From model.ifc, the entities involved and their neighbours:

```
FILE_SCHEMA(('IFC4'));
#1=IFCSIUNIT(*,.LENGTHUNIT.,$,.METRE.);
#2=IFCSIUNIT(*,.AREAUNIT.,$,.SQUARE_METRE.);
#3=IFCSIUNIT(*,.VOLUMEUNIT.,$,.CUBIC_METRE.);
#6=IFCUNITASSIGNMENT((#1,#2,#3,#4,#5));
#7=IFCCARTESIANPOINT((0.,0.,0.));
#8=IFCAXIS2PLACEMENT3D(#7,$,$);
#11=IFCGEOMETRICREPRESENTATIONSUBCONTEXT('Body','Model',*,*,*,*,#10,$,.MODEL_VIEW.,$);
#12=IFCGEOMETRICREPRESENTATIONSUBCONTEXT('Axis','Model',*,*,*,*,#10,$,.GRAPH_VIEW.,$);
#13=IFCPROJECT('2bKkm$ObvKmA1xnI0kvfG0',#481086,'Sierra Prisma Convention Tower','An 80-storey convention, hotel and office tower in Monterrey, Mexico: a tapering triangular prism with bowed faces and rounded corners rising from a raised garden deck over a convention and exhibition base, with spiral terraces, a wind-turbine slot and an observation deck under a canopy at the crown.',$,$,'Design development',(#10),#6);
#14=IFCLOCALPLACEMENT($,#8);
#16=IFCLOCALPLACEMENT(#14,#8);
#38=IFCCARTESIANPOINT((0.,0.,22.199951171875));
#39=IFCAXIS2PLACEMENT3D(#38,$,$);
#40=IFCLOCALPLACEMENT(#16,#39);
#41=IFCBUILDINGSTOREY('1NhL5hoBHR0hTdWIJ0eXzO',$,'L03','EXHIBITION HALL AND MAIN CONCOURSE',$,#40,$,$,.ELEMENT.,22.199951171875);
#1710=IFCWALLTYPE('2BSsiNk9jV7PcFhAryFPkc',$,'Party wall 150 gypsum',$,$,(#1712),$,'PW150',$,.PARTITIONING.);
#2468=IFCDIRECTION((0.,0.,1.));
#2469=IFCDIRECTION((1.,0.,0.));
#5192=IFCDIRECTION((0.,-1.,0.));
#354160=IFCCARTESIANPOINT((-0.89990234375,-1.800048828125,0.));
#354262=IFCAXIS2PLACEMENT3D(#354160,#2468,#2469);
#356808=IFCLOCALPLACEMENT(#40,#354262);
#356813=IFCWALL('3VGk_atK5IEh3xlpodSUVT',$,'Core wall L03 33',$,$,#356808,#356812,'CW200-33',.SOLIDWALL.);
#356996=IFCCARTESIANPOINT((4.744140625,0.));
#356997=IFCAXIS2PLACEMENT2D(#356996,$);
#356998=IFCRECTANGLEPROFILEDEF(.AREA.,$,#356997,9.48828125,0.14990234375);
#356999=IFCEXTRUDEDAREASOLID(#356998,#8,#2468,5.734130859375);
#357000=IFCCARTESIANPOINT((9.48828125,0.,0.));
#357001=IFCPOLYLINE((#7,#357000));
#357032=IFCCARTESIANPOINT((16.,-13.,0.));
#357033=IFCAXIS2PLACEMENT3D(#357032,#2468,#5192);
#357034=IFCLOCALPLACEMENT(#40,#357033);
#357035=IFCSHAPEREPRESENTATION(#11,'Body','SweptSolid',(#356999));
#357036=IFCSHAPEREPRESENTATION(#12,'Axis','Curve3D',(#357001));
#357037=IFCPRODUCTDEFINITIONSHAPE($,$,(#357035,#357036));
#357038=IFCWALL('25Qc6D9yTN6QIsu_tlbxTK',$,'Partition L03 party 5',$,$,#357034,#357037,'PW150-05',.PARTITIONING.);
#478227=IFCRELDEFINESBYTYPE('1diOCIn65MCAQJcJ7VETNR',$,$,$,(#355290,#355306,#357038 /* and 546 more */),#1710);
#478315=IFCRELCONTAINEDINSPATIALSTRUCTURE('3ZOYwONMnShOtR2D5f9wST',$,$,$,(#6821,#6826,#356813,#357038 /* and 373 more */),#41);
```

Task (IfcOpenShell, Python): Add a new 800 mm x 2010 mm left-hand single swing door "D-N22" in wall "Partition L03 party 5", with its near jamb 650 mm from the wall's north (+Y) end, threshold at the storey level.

```python
import numpy as np
import ifcopenshell
import ifcopenshell.api.feature
import ifcopenshell.api.geometry
import ifcopenshell.api.root
import ifcopenshell.api.spatial
import ifcopenshell.geom
import ifcopenshell.util.element
import ifcopenshell.util.placement
import ifcopenshell.util.representation
import ifcopenshell.util.shape
import ifcopenshell.util.unit

model = ifcopenshell.open("model.ifc")
unit_scale = ifcopenshell.util.unit.calculate_unit_scale(model)
settings = ifcopenshell.geom.settings()


def volume(element):
    """Net volume in cubic metres, openings subtracted."""
    shape = ifcopenshell.geom.create_shape(settings, element)
    return ifcopenshell.util.shape.get_volume(shape.geometry)


wall = model.by_guid("25Qc6D9yTN6QIsu_tlbxTK")
storey = ifcopenshell.util.element.get_container(wall, ifc_class="IfcBuildingStorey")
context = ifcopenshell.util.representation.get_context(model, "Model", "Body", "MODEL_VIEW")
before = volume(wall)

width, height, from_end, sill = 0.8, 2.01, 0.65, 0.0  # metres

# The wall runs along its own X axis, and the end named is its -X end.
wall_shape = ifcopenshell.geom.create_shape(settings, wall)
x, y, z = ifcopenshell.util.shape.get_vertices(wall_shape.geometry).T
start = x.min() + from_end
face, thickness = float(y.min()), float(y.max() - y.min())
wall_matrix = ifcopenshell.util.placement.get_local_placement(wall.ObjectPlacement)
level = ifcopenshell.util.placement.get_local_placement(storey.ObjectPlacement)[2, 3]


def in_wall(x, y):
    """Placement at x, y metres in the wall's axes, at sill height."""
    matrix = wall_matrix.copy()
    matrix[:, 3] = wall_matrix @ np.array([x / unit_scale, y / unit_scale, 0.0, 1.0])
    matrix[2, 3] = level + sill / unit_scale
    return matrix


# Opening: a box that overshoots both wall faces by 50 mm.
opening = ifcopenshell.api.root.create_entity(model, ifc_class="IfcOpeningElement", predefined_type="OPENING")
box = ifcopenshell.api.geometry.add_wall_representation(
    model, context=context, length=width, height=height, thickness=thickness + 0.1
)
ifcopenshell.api.geometry.assign_representation(model, product=opening, representation=box)
ifcopenshell.api.geometry.edit_object_placement(model, product=opening, matrix=in_wall(start, face - 0.05), is_si=False)
ifcopenshell.api.feature.add_feature(model, feature=opening, element=wall)

door = ifcopenshell.api.root.create_entity(model, ifc_class="IfcDoor", name="D-N22", predefined_type="DOOR")
door.OverallWidth, door.OverallHeight = width / unit_scale, height / unit_scale
door.OperationType = "SINGLE_SWING_LEFT"
body = ifcopenshell.api.geometry.add_door_representation(
    model,
    context=context,
    overall_width=door.OverallWidth,
    overall_height=door.OverallHeight,
    operation_type="SINGLE_SWING_LEFT",
    lining_properties={"LiningDepth": thickness / unit_scale, "ThresholdDepth": thickness / unit_scale},
)
ifcopenshell.api.geometry.assign_representation(model, product=door, representation=body)
ifcopenshell.api.spatial.assign_container(model, products=[door], relating_structure=storey)
ifcopenshell.api.feature.add_filling(model, opening=opening, element=door)

# The lining spans the wall, so the door starts at the wall face.
ifcopenshell.api.geometry.edit_object_placement(model, product=door, matrix=in_wall(start, face), is_si=False)

after = volume(wall)

print(f"wall volume {before:.3f} -> {after:.3f} m3")

model.write("model_v2.ifc")
```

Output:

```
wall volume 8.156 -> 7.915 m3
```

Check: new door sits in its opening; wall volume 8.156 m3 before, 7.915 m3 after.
